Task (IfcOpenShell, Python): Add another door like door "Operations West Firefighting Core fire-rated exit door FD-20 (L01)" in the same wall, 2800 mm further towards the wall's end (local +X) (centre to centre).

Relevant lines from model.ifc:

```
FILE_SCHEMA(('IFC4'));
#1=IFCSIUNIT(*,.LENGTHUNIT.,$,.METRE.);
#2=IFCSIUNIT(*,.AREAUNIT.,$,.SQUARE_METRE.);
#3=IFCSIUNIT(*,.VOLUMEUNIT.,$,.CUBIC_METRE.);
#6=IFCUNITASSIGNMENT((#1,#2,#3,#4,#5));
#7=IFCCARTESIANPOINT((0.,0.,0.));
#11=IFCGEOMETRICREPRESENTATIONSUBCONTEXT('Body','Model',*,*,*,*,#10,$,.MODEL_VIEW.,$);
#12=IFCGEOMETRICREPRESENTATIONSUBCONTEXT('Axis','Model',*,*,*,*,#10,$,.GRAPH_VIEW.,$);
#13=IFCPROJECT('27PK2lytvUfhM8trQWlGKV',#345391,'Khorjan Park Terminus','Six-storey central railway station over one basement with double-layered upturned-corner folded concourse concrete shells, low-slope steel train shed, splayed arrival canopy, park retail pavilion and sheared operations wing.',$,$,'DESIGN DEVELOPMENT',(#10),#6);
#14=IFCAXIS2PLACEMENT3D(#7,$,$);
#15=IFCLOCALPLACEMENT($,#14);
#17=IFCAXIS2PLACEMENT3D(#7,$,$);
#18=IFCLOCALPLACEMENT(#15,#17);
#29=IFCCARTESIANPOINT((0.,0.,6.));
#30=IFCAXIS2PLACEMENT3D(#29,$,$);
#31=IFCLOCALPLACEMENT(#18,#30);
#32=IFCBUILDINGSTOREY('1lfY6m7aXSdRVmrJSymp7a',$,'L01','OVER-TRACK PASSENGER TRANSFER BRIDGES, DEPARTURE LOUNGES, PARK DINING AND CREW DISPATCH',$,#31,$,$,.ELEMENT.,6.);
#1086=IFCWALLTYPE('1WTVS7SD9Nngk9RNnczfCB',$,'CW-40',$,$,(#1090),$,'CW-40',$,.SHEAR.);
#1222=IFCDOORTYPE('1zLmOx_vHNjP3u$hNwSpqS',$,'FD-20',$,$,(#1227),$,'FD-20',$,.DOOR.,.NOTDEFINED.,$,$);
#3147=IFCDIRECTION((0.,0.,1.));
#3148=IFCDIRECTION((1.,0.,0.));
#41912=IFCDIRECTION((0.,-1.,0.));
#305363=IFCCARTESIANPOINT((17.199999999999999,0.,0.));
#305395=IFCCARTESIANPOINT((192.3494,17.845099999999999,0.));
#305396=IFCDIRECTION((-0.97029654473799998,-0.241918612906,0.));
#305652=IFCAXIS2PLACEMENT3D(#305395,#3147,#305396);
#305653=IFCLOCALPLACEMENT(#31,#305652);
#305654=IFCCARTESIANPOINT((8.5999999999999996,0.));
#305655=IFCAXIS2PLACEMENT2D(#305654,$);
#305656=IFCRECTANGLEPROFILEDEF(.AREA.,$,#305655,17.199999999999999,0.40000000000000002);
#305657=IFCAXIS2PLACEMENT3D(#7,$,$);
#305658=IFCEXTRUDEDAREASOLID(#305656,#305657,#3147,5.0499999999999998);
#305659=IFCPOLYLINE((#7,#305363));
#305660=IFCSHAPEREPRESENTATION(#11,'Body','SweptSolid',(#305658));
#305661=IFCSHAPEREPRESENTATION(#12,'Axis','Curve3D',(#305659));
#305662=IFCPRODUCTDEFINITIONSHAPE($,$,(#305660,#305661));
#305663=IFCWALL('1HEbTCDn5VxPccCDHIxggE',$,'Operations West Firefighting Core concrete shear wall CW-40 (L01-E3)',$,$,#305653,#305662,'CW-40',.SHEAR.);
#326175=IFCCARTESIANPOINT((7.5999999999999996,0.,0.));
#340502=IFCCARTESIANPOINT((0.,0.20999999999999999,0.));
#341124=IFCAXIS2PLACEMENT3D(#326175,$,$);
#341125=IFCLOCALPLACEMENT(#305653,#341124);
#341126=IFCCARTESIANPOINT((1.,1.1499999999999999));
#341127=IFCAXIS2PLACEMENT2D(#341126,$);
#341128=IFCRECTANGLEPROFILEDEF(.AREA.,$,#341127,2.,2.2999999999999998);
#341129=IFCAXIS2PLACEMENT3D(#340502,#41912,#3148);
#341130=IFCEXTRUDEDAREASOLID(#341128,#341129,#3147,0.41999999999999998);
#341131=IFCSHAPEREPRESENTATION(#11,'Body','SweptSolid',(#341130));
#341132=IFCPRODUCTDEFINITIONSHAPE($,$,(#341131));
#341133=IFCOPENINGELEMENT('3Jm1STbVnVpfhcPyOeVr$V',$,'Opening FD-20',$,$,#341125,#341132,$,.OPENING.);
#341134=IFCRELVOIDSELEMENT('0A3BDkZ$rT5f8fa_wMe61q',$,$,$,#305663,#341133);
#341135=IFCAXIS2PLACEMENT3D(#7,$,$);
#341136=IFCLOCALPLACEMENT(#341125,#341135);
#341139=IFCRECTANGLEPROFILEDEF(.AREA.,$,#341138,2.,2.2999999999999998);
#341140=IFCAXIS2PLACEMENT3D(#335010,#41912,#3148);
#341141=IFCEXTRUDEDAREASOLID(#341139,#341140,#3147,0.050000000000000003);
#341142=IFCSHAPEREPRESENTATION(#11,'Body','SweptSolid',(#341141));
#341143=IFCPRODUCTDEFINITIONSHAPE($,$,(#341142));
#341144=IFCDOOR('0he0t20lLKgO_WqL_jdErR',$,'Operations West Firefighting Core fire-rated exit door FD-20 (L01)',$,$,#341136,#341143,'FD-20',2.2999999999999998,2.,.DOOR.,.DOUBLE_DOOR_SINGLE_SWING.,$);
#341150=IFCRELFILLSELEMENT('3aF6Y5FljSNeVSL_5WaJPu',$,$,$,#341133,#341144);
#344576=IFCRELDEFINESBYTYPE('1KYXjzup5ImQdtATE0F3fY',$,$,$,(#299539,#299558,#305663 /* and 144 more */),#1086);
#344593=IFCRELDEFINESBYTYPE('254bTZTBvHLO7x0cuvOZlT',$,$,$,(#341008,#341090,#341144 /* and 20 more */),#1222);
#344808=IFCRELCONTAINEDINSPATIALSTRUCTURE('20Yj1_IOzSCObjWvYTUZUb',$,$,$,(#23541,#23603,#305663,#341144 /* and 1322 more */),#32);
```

```python
import ifcopenshell
import ifcopenshell.api.feature
import ifcopenshell.api.geometry
import ifcopenshell.api.root
import ifcopenshell.geom
import ifcopenshell.util.element
import ifcopenshell.util.placement
import ifcopenshell.util.shape

model = ifcopenshell.open("model.ifc")
settings = ifcopenshell.geom.settings()


def volume(element):
    """Net volume in cubic metres, openings subtracted."""
    shape = ifcopenshell.geom.create_shape(settings, element)
    return ifcopenshell.util.shape.get_volume(shape.geometry)


door = model.by_guid("0he0t20lLKgO_WqL_jdErR")
opening = door.FillsVoids[0].RelatingOpeningElement
wall = opening.VoidsElements[0].RelatingBuildingElement
before = volume(wall)
shift = ifcopenshell.util.placement.get_local_placement(wall.ObjectPlacement)[:3, 0] * 2.8

# copy_class copies the void relationship, type, container and properties, but no geometry.
new_opening = ifcopenshell.api.root.copy_class(model, product=opening)
new_opening.Representation = ifcopenshell.util.element.copy_deep(
    model, opening.Representation, exclude=["IfcGeometricRepresentationContext", "IfcRepresentationMap"]
)
new_door = ifcopenshell.api.root.copy_class(model, product=door)
new_door.Representation = ifcopenshell.util.element.copy_deep(
    model, door.Representation, exclude=["IfcGeometricRepresentationContext", "IfcRepresentationMap"]
)
new_door.Tag = None
ifcopenshell.api.feature.add_filling(model, opening=new_opening, element=new_door)

for old, new in ((opening, new_opening), (door, new_door)):
    matrix = ifcopenshell.util.placement.get_local_placement(old.ObjectPlacement)
    matrix[:3, 3] += shift
    ifcopenshell.api.geometry.edit_object_placement(model, product=new, matrix=matrix, is_si=False)

after = volume(wall)

print(f"wall volume {before:.3f} -> {after:.3f} m3")

model.write("model_edited.ifc")
```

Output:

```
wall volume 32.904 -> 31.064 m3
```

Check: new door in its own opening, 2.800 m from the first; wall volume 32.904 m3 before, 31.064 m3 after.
